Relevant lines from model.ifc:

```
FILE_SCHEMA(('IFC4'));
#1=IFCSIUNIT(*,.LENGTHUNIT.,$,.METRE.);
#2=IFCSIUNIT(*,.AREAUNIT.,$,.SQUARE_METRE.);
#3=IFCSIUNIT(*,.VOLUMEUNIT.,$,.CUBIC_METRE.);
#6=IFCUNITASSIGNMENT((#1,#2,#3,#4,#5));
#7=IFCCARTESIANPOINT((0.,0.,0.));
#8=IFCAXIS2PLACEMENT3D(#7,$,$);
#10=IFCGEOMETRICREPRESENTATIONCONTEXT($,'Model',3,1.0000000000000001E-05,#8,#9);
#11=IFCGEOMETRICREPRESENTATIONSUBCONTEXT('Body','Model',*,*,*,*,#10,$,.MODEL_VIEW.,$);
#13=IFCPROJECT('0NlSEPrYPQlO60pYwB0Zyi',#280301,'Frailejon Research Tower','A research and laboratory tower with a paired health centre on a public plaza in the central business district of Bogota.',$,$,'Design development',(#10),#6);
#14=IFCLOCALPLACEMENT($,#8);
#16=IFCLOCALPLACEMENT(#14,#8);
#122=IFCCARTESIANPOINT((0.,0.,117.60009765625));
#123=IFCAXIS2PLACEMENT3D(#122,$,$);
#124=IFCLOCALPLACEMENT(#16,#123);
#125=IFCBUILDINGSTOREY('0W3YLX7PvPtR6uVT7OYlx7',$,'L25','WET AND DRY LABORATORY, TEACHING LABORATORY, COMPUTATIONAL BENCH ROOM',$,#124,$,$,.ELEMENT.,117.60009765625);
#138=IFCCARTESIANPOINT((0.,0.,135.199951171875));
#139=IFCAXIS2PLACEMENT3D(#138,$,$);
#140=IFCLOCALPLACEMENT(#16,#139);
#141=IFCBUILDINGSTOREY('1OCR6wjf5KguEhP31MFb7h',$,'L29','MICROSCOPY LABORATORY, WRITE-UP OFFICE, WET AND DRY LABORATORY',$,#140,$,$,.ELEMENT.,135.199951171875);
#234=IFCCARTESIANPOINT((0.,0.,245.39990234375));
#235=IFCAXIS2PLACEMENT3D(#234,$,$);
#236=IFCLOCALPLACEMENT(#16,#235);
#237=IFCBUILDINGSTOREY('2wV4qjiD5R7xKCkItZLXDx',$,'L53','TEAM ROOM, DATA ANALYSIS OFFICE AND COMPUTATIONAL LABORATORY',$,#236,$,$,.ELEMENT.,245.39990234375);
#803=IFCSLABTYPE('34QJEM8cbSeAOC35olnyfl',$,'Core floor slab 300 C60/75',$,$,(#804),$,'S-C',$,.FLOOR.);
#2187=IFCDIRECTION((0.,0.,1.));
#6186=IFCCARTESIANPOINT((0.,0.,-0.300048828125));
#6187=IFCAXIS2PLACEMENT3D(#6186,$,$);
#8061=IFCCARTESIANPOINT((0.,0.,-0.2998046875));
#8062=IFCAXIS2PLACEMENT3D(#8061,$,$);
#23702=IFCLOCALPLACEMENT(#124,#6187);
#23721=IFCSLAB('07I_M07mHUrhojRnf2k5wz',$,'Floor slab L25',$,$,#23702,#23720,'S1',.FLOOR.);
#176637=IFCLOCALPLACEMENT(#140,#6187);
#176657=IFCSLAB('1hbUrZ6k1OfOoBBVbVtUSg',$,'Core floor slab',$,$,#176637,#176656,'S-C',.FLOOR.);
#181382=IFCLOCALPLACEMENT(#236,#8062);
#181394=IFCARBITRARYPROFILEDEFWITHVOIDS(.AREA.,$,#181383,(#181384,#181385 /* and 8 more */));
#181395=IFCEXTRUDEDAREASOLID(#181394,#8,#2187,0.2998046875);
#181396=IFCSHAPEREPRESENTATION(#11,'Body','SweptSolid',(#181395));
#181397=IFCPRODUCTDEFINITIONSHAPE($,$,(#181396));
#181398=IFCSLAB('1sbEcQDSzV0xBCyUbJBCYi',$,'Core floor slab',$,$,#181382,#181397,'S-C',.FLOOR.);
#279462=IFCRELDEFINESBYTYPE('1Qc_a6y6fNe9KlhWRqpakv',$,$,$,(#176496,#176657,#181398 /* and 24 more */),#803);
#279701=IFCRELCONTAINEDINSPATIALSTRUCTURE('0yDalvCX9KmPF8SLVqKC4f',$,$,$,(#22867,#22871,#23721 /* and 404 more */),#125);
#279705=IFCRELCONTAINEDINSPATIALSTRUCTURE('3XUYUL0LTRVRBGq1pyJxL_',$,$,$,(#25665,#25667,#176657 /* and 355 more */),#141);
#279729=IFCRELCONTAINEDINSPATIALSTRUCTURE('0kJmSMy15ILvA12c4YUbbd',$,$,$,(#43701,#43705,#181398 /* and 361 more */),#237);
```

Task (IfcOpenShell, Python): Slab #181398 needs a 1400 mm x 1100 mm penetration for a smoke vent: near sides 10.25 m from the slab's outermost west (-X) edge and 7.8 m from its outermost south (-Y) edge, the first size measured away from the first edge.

```python
import numpy as np
import ifcopenshell
import ifcopenshell.api.feature
import ifcopenshell.api.geometry
import ifcopenshell.api.root
import ifcopenshell.geom
import ifcopenshell.util.placement
import ifcopenshell.util.representation
import ifcopenshell.util.shape
import ifcopenshell.util.unit

model = ifcopenshell.open("model.ifc")
unit_scale = ifcopenshell.util.unit.calculate_unit_scale(model)
settings = ifcopenshell.geom.settings()


def volume(element):
    """Net volume in cubic metres, openings subtracted."""
    shape = ifcopenshell.geom.create_shape(settings, element)
    return ifcopenshell.util.shape.get_volume(shape.geometry)


slab = model.by_guid("1sbEcQDSzV0xBCyUbJBCYi")
before = volume(slab)

# Extent in the slab's own axes, in metres. The edges named are its -X and -Y sides.
slab_shape = ifcopenshell.geom.create_shape(settings, slab)
vertices = ifcopenshell.util.shape.get_vertices(slab_shape.geometry)
x_min, y_min, bottom = vertices.min(axis=0)
top = vertices[:, 2].max()

opening = ifcopenshell.api.root.create_entity(model, ifc_class="IfcOpeningElement", name="Smoke vent opening", predefined_type="OPENING")
context = ifcopenshell.util.representation.get_context(model, "Model", "Body", "MODEL_VIEW")
width, depth = 1.4, 1.1
outline = [(0.0, 0.0), (width, 0.0), (width, depth), (0.0, depth), (0.0, 0.0)]
# Overshoot both faces by 50 mm so the cut is clean.
shape = ifcopenshell.api.geometry.add_slab_representation(
    model, context=context, depth=top - bottom + 0.1, polyline=outline
)
ifcopenshell.api.geometry.assign_representation(model, product=opening, representation=shape)

matrix = ifcopenshell.util.placement.get_local_placement(slab.ObjectPlacement)
matrix[:, 3] = matrix @ np.append(np.array([x_min + 10.25, y_min + 7.8, bottom - 0.05]) / unit_scale, 1.0)
ifcopenshell.api.geometry.edit_object_placement(model, product=opening, matrix=matrix, is_si=False)
ifcopenshell.api.feature.add_feature(model, feature=opening, element=slab)

after = volume(slab)

print(f"slab volume {before:.3f} -> {after:.3f} m3")

model.write("model_v2.ifc")
```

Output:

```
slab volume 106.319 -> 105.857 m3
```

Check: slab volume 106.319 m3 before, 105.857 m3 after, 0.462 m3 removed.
